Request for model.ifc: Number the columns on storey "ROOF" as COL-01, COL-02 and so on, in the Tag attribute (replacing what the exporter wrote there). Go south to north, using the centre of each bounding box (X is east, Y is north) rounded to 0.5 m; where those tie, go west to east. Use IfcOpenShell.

First a look at what the model holds.

```python
import ifcopenshell
import ifcopenshell.util.element
import ifcopenshell.util.placement

model = ifcopenshell.open("model.ifc")
print(model.schema)
storey = next(s for s in model.by_type("IfcBuildingStorey") if s.Name == "ROOF")
columns = [e for e in ifcopenshell.util.element.get_decomposition(storey) if e.is_a("IfcColumn")]
for e in sorted(columns, key=lambda e: e.id()):
    origin = ifcopenshell.util.placement.get_local_placement(e.ObjectPlacement)[:3, 3]
    print(e.id(), e.Tag, e.Name, origin.round(2) + 0.0, sep=" | ")
```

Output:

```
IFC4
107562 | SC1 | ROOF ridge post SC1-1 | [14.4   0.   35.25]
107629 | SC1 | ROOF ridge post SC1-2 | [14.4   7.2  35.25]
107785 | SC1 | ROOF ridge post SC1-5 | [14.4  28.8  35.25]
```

```python
import ifcopenshell
import ifcopenshell.geom
import ifcopenshell.util.element
import ifcopenshell.util.shape

model = ifcopenshell.open("model.ifc")
settings = ifcopenshell.geom.settings()
settings.set("use-world-coords", True)


def centre(element):
    shape = ifcopenshell.geom.create_shape(settings, element)
    return ifcopenshell.util.shape.get_bbox_centroid(shape.geometry)


storey = next(s for s in model.by_type("IfcBuildingStorey") if s.Name == "ROOF")
columns = [e for e in ifcopenshell.util.element.get_decomposition(storey) if e.is_a("IfcColumn")]

# Insertion points can sit at a corner or the storey origin, so sort by the geometry (in metres).
centres = {e: centre(e) for e in columns}
columns.sort(key=lambda e: (round(centres[e][1] / 0.5), centres[e][0]))

for i, e in enumerate(columns, start=1):
    number = f"COL-{i:02d}"
    e.Tag = number
    print(e.id(), number)

model.write("model_rev.ifc")
```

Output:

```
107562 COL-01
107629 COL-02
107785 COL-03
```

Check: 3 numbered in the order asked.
